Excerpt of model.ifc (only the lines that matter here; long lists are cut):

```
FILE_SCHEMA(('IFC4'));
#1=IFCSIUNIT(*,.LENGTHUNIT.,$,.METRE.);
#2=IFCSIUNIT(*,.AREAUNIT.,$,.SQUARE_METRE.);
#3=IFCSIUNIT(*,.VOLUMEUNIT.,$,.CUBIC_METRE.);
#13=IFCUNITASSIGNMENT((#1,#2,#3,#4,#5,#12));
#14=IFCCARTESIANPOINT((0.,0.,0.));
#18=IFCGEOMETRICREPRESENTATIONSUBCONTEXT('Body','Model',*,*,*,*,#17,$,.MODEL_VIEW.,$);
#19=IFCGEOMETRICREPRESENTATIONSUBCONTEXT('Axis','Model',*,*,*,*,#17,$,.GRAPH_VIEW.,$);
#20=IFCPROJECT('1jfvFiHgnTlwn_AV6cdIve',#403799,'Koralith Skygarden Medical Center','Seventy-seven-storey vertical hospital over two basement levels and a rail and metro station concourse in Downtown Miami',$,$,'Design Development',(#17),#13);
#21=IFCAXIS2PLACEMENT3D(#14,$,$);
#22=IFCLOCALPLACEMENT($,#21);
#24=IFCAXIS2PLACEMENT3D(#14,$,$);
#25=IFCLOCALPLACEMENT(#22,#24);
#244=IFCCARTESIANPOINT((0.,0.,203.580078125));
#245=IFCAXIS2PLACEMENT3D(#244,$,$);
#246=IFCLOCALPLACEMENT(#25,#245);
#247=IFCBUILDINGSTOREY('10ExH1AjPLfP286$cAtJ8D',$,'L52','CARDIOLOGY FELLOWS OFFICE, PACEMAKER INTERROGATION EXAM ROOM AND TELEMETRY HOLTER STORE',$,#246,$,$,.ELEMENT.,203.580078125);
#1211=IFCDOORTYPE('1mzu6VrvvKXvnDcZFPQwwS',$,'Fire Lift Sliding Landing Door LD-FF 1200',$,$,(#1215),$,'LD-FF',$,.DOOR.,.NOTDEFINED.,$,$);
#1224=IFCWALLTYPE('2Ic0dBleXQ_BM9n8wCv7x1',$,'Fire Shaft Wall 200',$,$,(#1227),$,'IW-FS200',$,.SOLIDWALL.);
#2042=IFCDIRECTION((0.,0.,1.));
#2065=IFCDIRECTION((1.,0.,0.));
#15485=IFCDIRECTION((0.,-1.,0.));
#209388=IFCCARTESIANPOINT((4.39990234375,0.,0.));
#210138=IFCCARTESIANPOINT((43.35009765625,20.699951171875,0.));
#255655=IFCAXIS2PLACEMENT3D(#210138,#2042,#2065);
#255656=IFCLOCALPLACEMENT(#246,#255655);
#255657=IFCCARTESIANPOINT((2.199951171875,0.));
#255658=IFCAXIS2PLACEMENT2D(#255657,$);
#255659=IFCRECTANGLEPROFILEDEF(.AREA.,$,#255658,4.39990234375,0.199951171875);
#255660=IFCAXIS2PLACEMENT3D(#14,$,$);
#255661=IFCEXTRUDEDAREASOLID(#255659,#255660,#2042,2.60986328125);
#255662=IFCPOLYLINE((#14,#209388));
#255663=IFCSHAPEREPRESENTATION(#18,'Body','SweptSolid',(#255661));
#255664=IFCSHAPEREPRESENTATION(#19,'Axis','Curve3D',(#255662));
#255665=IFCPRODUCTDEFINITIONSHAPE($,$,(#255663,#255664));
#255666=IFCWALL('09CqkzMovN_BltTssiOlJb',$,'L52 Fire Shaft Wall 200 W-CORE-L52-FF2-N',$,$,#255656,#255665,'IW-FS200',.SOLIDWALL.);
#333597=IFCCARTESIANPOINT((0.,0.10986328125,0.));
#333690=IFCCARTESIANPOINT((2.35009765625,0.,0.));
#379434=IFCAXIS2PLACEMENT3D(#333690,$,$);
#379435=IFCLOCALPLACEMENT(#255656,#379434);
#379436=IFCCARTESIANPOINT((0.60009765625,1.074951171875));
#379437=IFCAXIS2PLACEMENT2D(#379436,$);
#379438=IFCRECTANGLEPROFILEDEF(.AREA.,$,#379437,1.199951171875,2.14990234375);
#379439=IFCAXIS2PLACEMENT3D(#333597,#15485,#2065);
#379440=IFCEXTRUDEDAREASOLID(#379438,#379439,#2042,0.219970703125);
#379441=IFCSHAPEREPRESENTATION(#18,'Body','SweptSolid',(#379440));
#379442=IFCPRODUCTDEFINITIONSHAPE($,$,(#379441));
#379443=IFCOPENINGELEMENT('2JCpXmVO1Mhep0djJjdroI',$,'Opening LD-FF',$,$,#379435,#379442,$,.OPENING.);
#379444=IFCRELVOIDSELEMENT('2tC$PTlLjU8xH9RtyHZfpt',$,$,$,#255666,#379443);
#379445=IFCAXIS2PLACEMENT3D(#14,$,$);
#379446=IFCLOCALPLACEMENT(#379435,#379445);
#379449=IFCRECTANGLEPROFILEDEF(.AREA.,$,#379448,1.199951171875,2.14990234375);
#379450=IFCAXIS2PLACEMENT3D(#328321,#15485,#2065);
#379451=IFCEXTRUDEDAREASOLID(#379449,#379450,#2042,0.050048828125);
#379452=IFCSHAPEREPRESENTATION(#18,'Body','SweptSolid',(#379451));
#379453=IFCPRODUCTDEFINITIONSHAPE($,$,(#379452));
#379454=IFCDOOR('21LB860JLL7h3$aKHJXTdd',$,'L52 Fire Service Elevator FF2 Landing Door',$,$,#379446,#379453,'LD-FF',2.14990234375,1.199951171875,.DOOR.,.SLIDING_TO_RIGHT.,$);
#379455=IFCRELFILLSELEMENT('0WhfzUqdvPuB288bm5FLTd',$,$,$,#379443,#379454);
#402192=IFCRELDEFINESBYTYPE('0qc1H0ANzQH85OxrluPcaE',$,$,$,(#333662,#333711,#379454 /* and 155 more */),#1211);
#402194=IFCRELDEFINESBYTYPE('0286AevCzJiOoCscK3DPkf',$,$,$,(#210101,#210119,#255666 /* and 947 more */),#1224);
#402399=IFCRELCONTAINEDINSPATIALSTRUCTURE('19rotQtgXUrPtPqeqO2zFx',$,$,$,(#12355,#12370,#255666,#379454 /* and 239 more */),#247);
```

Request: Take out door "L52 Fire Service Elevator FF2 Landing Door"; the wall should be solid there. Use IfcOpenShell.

```python
import ifcopenshell
import ifcopenshell.api.feature
import ifcopenshell.api.root
import ifcopenshell.geom
import ifcopenshell.util.shape

model = ifcopenshell.open("model.ifc")
settings = ifcopenshell.geom.settings()


def volume(element):
    """Net volume in cubic metres, openings subtracted."""
    shape = ifcopenshell.geom.create_shape(settings, element)
    return ifcopenshell.util.shape.get_volume(shape.geometry)


door = model.by_guid("21LB860JLL7h3$aKHJXTdd")
opening = door.FillsVoids[0].RelatingOpeningElement
wall = opening.VoidsElements[0].RelatingBuildingElement
before = volume(wall)

ifcopenshell.api.root.remove_product(model, product=door)
ifcopenshell.api.feature.remove_feature(model, feature=opening)

after = volume(wall)

print(f"wall volume {before:.3f} -> {after:.3f} m3")

model.write("model-out.ifc")
```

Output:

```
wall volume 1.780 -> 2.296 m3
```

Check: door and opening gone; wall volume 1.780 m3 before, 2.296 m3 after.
